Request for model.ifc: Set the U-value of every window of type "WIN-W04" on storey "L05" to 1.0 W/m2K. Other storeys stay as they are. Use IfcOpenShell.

First a look at what the model holds.

```python
import ifcopenshell
import ifcopenshell.util.element

model = ifcopenshell.open("model.ifc")
print(model.schema)
storey = next(s for s in model.by_type("IfcBuildingStorey") if s.Name == "L05")
windows = [e for e in ifcopenshell.util.element.get_decomposition(storey) if e.is_a("IfcWindow")]
seen = {}
for e in windows:
    element_type = ifcopenshell.util.element.get_type(e)
    key = (element_type.Name if element_type != e and element_type else None, ifcopenshell.util.element.get_pset(e, "Pset_WindowCommon", "ThermalTransmittance"))
    seen[key] = seen.get(key, 0) + 1
for (name, value), count in sorted(seen.items(), key=str):
    print(count, "x", name, "|", value)
```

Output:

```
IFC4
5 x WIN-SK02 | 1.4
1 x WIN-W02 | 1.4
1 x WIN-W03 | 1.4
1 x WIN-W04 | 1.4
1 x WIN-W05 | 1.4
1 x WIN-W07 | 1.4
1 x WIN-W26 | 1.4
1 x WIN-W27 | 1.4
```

```python
import ifcopenshell
import ifcopenshell.api.pset
import ifcopenshell.util.element

model = ifcopenshell.open("model.ifc")

storey = next(s for s in model.by_type("IfcBuildingStorey") if s.Name == "L05")
windows = [e for e in ifcopenshell.util.element.get_decomposition(storey) if e.is_a("IfcWindow")]

count = 0
for e in windows:
    element_type = ifcopenshell.util.element.get_type(e)
    if element_type in (None, e) or element_type.Name != "WIN-W04":
        continue
    # add_pset returns the element's existing set when there is one.
    pset = ifcopenshell.api.pset.add_pset(model, product=e, name="Pset_WindowCommon")
    ifcopenshell.api.pset.edit_pset(model, pset=pset, properties={"ThermalTransmittance": 1.0})
    count += 1

print(count, "windows updated")

model.write("model_rev.ifc")
```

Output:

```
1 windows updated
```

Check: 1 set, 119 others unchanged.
